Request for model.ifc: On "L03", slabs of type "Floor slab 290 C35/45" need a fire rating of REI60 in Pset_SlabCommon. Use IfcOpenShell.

First a look at what the model holds.

```python
import ifcopenshell
import ifcopenshell.util.element

model = ifcopenshell.open("model.ifc")
print(model.schema)
storey = next(s for s in model.by_type("IfcBuildingStorey") if s.Name == "L03")
slabs = [e for e in ifcopenshell.util.element.get_decomposition(storey) if e.is_a("IfcSlab")]
seen = {}
for e in slabs:
    element_type = ifcopenshell.util.element.get_type(e)
    key = (element_type.Name if element_type != e and element_type else None, ifcopenshell.util.element.get_pset(e, "Pset_SlabCommon", "FireRating"))
    seen[key] = seen.get(key, 0) + 1
for (name, value), count in sorted(seen.items(), key=str):
    print(count, "x", name, "|", value)
```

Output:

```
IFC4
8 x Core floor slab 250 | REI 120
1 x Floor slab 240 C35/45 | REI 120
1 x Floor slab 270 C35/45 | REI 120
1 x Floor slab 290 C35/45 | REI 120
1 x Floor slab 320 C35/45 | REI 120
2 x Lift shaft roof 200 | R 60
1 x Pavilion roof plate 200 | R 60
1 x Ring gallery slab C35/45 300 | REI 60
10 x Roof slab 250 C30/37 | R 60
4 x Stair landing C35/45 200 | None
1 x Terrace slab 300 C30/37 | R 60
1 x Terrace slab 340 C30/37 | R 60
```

```python
import ifcopenshell
import ifcopenshell.api.pset
import ifcopenshell.util.element

model = ifcopenshell.open("model.ifc")

storey = next(s for s in model.by_type("IfcBuildingStorey") if s.Name == "L03")
slabs = [e for e in ifcopenshell.util.element.get_decomposition(storey) if e.is_a("IfcSlab")]

count = 0
for e in slabs:
    element_type = ifcopenshell.util.element.get_type(e)
    if element_type in (None, e) or element_type.Name != "Floor slab 290 C35/45":
        continue
    # add_pset returns the element's existing set when there is one.
    pset = ifcopenshell.api.pset.add_pset(model, product=e, name="Pset_SlabCommon")
    ifcopenshell.api.pset.edit_pset(model, pset=pset, properties={"FireRating": "REI60"})
    count += 1

print(count, "slabs updated")

model.write("model_v2.ifc")
```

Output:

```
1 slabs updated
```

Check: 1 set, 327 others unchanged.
